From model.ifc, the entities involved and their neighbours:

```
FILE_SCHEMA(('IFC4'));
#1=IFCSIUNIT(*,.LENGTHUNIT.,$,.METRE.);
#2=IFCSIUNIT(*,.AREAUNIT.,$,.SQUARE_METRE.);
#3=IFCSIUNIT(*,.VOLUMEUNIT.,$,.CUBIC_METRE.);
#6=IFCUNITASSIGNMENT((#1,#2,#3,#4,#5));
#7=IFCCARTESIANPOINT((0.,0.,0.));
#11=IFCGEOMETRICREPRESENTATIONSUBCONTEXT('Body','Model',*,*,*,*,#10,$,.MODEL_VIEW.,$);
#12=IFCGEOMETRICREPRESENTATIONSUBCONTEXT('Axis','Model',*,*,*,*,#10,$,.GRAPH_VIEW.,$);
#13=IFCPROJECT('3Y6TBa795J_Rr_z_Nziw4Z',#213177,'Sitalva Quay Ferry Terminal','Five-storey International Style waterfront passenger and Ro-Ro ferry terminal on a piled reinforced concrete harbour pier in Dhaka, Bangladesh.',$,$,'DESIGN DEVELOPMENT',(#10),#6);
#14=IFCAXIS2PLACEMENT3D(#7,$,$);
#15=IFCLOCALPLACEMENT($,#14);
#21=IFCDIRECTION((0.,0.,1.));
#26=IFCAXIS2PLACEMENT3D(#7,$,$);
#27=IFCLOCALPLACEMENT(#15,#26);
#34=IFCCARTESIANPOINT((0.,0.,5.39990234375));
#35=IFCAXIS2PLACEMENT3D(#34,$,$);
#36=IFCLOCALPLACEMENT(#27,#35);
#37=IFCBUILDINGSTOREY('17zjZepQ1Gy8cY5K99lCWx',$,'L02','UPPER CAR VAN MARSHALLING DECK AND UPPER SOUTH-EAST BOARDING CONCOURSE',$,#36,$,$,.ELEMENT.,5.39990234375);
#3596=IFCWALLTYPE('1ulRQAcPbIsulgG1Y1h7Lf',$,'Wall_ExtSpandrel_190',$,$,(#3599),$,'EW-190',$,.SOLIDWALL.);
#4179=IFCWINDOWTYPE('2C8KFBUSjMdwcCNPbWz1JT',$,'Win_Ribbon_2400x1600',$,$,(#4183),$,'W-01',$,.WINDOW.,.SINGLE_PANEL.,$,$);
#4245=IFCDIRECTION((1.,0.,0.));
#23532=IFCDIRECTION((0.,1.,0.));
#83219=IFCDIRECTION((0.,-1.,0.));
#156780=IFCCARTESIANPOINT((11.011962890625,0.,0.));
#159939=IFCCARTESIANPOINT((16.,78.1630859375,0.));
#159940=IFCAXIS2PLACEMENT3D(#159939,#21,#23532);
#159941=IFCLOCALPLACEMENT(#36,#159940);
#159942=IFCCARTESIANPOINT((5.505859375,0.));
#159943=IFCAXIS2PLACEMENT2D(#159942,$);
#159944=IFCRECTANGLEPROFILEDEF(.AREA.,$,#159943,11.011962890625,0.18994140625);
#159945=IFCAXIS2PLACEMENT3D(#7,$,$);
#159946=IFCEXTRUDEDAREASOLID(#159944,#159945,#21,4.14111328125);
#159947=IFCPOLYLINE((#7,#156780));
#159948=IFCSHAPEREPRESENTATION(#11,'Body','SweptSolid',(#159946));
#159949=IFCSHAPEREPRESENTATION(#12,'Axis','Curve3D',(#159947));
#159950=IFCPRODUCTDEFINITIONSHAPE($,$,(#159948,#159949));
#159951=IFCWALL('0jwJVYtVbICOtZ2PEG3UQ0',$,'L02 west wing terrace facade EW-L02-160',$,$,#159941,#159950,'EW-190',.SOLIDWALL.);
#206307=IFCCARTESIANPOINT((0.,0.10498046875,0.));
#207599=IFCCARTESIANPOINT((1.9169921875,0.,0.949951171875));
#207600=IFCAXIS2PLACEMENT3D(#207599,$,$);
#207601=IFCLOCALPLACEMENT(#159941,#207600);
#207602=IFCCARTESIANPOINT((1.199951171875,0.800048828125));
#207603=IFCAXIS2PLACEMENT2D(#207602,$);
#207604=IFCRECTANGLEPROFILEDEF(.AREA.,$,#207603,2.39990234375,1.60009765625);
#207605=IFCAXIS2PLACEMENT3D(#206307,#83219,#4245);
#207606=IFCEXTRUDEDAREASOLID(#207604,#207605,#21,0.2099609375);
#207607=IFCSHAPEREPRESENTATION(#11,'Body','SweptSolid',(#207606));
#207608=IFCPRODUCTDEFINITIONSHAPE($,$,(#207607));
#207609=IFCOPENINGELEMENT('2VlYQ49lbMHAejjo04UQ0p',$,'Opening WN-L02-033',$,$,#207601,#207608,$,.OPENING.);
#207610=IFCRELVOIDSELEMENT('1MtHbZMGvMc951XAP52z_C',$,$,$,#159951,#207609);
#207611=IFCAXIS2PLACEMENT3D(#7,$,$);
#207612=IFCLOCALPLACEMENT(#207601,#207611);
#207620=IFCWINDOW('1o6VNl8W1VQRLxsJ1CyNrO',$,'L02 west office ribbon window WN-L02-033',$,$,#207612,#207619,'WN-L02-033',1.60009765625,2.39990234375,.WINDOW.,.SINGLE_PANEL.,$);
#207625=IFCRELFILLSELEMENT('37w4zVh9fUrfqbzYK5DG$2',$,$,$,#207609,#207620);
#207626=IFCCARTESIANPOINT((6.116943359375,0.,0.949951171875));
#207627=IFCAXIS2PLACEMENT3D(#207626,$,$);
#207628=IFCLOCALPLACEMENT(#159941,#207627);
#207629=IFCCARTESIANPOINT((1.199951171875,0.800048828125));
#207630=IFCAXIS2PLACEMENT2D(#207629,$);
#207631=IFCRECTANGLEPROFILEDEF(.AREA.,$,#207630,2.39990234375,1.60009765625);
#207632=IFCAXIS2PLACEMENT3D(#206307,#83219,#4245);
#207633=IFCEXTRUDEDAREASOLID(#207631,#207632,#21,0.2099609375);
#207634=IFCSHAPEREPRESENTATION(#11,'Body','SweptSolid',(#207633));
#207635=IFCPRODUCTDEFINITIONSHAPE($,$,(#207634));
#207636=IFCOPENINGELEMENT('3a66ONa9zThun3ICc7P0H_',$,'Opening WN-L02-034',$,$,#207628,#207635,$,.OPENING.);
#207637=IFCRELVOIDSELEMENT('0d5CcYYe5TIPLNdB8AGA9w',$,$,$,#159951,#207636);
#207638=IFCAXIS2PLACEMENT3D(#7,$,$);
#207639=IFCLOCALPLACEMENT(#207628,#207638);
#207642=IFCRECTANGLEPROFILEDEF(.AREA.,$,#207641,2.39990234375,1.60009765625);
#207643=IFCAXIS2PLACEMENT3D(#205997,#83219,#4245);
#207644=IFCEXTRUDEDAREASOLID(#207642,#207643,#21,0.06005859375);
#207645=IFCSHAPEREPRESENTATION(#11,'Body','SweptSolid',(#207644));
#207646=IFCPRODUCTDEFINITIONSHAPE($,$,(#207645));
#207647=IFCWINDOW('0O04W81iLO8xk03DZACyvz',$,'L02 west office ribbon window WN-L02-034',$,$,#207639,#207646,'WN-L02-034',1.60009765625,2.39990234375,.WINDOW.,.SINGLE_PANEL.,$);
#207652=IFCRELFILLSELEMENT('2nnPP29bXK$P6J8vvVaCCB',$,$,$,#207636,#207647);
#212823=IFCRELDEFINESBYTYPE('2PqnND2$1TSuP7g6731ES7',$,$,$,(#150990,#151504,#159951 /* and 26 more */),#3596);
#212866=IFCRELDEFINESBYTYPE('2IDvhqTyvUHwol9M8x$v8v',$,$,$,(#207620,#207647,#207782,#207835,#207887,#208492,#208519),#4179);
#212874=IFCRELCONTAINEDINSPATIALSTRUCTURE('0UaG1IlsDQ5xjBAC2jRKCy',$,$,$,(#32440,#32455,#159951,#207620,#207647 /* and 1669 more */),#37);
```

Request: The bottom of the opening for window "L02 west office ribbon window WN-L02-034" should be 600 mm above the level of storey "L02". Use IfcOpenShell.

```python
import numpy as np
import ifcopenshell
import ifcopenshell.api.geometry
import ifcopenshell.geom
import ifcopenshell.util.element
import ifcopenshell.util.placement
import ifcopenshell.util.shape
import ifcopenshell.util.unit

model = ifcopenshell.open("model.ifc")
unit_scale = ifcopenshell.util.unit.calculate_unit_scale(model)

window = model.by_guid("0O04W81iLO8xk03DZACyvz")
opening = window.FillsVoids[0].RelatingOpeningElement
storey = ifcopenshell.util.element.get_container(window, ifc_class="IfcBuildingStorey")
level = ifcopenshell.util.placement.get_local_placement(storey.ObjectPlacement)[2, 3]

# The opening's origin need not be at the sill, so measure its lowest point.
shape = ifcopenshell.geom.create_shape(ifcopenshell.geom.settings(), opening)
bottom = ifcopenshell.util.shape.get_shape_bottom_elevation(shape, shape.geometry) / unit_scale
dz = level + 0.6 - bottom

shift = np.array([0.0, 0.0, dz])
# The window is placed relative to its opening, so it follows when the opening moves.
matrix = ifcopenshell.util.placement.get_local_placement(opening.ObjectPlacement)
matrix[:3, 3] += shift
ifcopenshell.api.geometry.edit_object_placement(
    model, product=opening, matrix=matrix, is_si=False, should_transform_children=True
)

print(f"moved by {dz * unit_scale:+.3f} m")

model.write("model_v2.ifc")
```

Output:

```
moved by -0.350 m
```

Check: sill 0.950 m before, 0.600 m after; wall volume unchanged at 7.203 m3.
